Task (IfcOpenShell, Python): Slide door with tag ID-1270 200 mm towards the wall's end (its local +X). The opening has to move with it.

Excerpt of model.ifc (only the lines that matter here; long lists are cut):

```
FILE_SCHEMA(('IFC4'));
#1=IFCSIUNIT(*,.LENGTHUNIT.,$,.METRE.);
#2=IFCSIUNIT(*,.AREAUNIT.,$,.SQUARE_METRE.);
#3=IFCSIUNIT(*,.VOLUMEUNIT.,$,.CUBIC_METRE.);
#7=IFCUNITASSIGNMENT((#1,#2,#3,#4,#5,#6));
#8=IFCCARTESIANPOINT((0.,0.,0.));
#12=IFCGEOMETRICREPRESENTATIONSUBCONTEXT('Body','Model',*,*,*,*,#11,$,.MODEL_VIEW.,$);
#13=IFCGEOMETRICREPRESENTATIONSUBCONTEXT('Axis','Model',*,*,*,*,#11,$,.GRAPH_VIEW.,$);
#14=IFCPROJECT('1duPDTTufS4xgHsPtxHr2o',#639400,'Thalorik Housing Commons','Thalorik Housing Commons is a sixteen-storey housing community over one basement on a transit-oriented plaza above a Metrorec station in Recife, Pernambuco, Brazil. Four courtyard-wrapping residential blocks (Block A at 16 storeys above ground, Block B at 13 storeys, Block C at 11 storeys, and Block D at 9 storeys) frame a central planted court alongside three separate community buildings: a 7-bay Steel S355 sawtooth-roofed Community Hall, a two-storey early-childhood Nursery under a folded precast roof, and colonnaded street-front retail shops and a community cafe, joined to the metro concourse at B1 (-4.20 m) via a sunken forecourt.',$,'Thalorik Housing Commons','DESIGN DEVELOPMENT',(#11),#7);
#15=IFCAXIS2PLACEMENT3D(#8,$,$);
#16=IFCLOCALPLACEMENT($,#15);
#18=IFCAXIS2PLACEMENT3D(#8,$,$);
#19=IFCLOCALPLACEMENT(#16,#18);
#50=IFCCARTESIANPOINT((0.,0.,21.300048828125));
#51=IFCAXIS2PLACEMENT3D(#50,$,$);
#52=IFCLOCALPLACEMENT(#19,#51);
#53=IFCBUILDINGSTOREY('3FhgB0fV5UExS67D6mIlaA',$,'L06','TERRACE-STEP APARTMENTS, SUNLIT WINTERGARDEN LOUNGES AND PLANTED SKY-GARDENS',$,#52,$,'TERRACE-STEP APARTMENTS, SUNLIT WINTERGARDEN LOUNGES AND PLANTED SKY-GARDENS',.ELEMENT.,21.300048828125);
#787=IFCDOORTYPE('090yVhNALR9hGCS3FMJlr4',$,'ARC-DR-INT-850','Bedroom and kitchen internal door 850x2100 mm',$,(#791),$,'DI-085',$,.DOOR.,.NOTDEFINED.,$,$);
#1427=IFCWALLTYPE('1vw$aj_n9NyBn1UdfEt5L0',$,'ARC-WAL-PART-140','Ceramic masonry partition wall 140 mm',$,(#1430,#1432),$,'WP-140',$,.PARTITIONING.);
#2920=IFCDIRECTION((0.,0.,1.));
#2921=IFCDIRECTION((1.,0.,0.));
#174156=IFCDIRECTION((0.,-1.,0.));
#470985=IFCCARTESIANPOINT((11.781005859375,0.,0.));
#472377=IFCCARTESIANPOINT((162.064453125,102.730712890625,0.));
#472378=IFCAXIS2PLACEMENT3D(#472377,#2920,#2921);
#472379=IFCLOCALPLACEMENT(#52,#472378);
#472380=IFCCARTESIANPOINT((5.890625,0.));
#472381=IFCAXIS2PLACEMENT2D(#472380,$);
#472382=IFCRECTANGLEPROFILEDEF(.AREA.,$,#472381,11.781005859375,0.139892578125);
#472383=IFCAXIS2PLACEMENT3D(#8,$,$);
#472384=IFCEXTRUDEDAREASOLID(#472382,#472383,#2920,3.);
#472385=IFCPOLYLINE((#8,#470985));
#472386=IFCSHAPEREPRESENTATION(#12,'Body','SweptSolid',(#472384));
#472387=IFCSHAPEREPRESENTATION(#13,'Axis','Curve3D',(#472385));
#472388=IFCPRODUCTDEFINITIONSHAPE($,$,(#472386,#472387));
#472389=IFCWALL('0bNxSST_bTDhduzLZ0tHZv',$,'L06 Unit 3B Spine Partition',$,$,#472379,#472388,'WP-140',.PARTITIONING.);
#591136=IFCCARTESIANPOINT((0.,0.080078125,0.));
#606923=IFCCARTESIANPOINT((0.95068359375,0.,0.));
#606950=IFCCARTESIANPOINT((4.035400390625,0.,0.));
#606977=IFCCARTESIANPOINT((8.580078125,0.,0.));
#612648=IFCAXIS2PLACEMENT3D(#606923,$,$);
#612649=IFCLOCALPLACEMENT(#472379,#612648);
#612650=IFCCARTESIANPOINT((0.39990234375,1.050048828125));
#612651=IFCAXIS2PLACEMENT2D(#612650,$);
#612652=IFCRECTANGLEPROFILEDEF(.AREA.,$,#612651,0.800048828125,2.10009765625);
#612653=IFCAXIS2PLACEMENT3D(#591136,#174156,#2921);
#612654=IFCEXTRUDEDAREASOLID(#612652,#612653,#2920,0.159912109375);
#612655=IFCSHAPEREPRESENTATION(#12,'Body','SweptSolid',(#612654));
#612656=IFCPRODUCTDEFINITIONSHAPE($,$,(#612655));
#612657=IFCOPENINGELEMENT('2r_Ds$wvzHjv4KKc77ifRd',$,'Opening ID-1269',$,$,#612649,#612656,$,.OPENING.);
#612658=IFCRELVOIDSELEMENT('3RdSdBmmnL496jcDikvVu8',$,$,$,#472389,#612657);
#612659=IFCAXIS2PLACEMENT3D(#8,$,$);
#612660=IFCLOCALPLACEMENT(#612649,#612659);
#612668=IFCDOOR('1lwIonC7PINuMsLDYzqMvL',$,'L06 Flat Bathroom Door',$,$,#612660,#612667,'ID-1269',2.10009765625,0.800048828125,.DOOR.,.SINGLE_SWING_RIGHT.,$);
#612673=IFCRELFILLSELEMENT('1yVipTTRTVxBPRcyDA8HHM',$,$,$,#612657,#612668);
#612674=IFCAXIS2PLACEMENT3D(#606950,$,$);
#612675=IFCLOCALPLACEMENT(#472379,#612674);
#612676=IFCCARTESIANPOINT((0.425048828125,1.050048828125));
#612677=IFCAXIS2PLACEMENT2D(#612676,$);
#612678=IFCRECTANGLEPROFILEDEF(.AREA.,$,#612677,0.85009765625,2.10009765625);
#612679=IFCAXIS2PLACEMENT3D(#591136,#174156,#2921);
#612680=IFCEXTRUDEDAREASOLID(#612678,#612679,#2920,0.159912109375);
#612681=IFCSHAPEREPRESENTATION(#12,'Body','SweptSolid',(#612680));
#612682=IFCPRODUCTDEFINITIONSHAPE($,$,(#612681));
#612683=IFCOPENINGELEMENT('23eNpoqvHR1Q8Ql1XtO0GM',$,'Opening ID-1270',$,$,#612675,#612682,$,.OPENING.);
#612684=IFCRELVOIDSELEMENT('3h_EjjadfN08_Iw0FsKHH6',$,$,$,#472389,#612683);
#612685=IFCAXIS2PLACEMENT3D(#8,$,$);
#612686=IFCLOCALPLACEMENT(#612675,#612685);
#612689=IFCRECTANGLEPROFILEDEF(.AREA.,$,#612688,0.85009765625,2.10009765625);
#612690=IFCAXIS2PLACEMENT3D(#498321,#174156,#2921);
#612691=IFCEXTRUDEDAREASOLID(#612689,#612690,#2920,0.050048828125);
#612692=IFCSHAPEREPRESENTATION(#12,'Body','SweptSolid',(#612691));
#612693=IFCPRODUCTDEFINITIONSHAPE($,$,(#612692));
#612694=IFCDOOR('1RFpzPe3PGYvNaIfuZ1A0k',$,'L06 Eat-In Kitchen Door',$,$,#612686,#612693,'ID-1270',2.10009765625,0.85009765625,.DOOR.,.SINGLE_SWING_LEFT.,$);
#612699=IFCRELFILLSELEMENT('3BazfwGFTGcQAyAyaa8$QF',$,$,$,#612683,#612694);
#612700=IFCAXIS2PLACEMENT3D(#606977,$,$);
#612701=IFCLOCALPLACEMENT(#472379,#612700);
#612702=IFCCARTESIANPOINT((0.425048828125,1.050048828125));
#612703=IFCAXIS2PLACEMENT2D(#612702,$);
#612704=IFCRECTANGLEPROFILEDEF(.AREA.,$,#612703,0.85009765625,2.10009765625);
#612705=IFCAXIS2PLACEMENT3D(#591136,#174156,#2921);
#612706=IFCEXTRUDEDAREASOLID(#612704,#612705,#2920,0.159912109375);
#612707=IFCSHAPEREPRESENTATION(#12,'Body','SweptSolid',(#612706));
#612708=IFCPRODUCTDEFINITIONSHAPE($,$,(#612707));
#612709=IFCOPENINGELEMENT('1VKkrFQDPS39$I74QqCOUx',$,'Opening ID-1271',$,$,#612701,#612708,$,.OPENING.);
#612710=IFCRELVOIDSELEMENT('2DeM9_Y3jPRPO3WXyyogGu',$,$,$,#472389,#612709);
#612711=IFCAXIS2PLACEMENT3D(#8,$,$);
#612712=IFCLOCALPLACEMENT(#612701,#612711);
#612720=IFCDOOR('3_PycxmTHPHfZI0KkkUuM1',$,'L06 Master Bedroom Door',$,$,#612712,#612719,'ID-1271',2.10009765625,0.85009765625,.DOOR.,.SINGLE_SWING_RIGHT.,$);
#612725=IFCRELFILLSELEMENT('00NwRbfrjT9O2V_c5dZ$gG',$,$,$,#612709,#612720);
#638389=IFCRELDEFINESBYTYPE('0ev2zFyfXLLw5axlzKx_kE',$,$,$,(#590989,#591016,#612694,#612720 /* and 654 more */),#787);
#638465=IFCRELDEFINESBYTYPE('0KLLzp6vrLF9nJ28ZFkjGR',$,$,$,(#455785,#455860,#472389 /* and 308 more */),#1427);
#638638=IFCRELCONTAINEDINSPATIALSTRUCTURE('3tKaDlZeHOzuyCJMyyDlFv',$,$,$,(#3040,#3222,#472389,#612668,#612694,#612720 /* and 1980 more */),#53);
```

```python
import ifcopenshell
import ifcopenshell.api.geometry
import ifcopenshell.util.placement
import ifcopenshell.util.unit

model = ifcopenshell.open("model.ifc")
unit_scale = ifcopenshell.util.unit.calculate_unit_scale(model)

door = model.by_guid("1RFpzPe3PGYvNaIfuZ1A0k")
opening = door.FillsVoids[0].RelatingOpeningElement
wall = opening.VoidsElements[0].RelatingBuildingElement

wall_matrix = ifcopenshell.util.placement.get_local_placement(wall.ObjectPlacement)
shift = wall_matrix[:3, 0] * 0.2 / unit_scale
before = ifcopenshell.util.placement.get_local_placement(door.ObjectPlacement)[:3, 3].copy()

# The door is placed relative to its opening, so it follows when the opening moves.
matrix = ifcopenshell.util.placement.get_local_placement(opening.ObjectPlacement)
matrix[:3, 3] += shift
ifcopenshell.api.geometry.edit_object_placement(
    model, product=opening, matrix=matrix, is_si=False, should_transform_children=True
)

after = ifcopenshell.util.placement.get_local_placement(door.ObjectPlacement)[:3, 3]
print("door moved by", (after - before).round(3) + 0.0)

model.write("model_v2.ifc")
```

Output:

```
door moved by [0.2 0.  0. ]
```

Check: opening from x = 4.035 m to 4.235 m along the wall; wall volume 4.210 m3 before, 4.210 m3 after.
